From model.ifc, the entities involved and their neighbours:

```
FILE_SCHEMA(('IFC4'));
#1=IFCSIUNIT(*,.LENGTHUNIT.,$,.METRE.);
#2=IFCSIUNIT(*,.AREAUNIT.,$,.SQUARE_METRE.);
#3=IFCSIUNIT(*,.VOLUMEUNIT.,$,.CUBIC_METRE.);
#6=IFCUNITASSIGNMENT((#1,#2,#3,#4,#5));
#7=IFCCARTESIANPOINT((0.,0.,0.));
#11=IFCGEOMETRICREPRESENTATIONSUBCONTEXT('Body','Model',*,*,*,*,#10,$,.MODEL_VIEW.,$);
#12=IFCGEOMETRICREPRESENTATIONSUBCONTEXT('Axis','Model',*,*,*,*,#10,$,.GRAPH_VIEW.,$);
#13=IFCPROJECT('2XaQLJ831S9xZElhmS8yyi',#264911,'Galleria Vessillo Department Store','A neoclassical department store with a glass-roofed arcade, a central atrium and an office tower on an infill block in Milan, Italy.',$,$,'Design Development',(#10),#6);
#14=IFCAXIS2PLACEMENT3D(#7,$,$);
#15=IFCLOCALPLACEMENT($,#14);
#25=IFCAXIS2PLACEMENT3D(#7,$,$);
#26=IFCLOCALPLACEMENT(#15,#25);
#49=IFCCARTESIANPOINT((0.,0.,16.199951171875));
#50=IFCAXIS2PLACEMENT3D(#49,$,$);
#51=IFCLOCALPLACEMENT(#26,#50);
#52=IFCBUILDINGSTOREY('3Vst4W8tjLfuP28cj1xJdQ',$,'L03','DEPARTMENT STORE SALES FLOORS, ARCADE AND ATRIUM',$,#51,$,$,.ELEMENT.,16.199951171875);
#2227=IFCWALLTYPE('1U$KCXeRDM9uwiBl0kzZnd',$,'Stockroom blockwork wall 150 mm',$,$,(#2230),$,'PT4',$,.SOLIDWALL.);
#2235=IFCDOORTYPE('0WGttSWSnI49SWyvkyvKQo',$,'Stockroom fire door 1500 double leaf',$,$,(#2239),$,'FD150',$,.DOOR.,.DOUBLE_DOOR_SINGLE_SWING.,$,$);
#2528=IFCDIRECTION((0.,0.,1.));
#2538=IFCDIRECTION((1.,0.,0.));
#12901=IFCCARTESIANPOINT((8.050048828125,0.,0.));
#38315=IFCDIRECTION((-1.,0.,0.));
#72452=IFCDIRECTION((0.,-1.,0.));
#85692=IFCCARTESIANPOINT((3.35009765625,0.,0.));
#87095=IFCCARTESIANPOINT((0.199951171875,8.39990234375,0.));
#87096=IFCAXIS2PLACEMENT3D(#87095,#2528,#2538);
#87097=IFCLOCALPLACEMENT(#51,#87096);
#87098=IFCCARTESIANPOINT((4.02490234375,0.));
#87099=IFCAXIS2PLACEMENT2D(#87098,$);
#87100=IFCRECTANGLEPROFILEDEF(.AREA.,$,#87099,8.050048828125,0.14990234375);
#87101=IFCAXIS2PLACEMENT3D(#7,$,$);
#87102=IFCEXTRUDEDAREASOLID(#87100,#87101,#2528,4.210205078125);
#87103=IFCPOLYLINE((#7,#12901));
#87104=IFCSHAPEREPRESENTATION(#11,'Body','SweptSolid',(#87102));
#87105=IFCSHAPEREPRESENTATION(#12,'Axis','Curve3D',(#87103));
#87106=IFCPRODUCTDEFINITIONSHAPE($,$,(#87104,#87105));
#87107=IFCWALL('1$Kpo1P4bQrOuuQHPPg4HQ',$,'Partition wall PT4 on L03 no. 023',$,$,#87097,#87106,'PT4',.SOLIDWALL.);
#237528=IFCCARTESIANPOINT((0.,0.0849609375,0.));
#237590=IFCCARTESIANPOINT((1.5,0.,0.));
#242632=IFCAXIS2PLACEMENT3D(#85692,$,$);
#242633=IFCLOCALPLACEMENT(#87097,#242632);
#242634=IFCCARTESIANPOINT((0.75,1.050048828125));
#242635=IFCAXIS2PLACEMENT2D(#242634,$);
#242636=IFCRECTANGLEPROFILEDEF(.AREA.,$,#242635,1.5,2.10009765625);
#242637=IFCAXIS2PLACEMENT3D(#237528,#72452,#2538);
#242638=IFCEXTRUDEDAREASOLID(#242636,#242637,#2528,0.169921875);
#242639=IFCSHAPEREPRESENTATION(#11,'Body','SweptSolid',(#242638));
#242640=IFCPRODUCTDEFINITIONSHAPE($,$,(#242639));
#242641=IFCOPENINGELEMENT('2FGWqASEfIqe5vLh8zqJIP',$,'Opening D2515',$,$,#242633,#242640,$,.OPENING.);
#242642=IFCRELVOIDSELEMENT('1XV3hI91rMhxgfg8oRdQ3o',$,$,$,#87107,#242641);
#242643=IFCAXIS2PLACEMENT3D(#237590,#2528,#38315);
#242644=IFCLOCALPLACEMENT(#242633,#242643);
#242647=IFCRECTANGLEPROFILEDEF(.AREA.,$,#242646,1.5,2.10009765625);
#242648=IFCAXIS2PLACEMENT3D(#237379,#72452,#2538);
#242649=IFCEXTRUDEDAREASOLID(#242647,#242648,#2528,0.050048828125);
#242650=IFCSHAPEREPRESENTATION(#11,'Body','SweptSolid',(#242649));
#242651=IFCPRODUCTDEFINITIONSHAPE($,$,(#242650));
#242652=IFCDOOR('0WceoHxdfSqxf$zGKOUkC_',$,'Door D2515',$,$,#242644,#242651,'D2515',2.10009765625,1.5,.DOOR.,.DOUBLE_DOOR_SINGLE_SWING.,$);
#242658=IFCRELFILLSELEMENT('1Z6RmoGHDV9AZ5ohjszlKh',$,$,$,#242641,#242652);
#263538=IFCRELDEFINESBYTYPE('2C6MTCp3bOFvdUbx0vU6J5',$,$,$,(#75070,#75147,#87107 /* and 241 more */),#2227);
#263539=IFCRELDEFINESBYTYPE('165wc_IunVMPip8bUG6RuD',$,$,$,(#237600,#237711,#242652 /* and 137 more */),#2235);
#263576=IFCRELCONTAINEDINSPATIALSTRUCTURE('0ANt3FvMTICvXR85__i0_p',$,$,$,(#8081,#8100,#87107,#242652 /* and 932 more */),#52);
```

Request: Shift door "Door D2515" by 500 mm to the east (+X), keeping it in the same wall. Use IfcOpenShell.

```python
import ifcopenshell
import ifcopenshell.api.geometry
import ifcopenshell.util.placement

model = ifcopenshell.open("model.ifc")

door = model.by_id(242652)
opening = door.FillsVoids[0].RelatingOpeningElement
wall = opening.VoidsElements[0].RelatingBuildingElement

wall_matrix = ifcopenshell.util.placement.get_local_placement(wall.ObjectPlacement)
shift = wall_matrix[:3, 0] * 0.5
before = ifcopenshell.util.placement.get_local_placement(door.ObjectPlacement)[:3, 3].copy()

# The door is placed relative to its opening, so it follows when the opening moves.
matrix = ifcopenshell.util.placement.get_local_placement(opening.ObjectPlacement)
matrix[:3, 3] += shift
ifcopenshell.api.geometry.edit_object_placement(
    model, product=opening, matrix=matrix, is_si=False, should_transform_children=True
)

after = ifcopenshell.util.placement.get_local_placement(door.ObjectPlacement)[:3, 3]
print("door moved by", (after - before).round(3) + 0.0)

model.write("model-out.ifc")
```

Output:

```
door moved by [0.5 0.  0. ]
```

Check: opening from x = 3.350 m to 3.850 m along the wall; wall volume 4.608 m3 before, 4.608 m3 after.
